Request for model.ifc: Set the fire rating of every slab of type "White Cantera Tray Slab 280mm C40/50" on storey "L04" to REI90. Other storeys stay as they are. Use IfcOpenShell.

First a look at what the model holds.

```python
import ifcopenshell
import ifcopenshell.util.element

model = ifcopenshell.open("model.ifc")
print(model.schema)
storey = next(s for s in model.by_type("IfcBuildingStorey") if s.Name == "L04")
slabs = [e for e in ifcopenshell.util.element.get_decomposition(storey) if e.is_a("IfcSlab")]
seen = {}
for e in slabs:
    element_type = ifcopenshell.util.element.get_type(e)
    key = (element_type.Name if element_type != e and element_type else None, ifcopenshell.util.element.get_pset(e, "Pset_SlabCommon", "FireRating"))
    seen[key] = seen.get(key, 0) + 1
for (name, value), count in sorted(seen.items(), key=str):
    print(count, "x", name, "|", value)
```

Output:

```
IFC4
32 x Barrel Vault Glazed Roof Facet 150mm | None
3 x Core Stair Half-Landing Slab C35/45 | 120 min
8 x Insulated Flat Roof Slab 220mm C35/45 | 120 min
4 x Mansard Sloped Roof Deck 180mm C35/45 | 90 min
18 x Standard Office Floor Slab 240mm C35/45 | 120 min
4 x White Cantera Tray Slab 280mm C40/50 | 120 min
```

```python
import ifcopenshell
import ifcopenshell.api.pset
import ifcopenshell.util.element

model = ifcopenshell.open("model.ifc")

storey = next(s for s in model.by_type("IfcBuildingStorey") if s.Name == "L04")
slabs = [e for e in ifcopenshell.util.element.get_decomposition(storey) if e.is_a("IfcSlab")]

count = 0
for e in slabs:
    element_type = ifcopenshell.util.element.get_type(e)
    if element_type in (None, e) or element_type.Name != "White Cantera Tray Slab 280mm C40/50":
        continue
    # add_pset returns the element's existing set when there is one.
    pset = ifcopenshell.api.pset.add_pset(model, product=e, name="Pset_SlabCommon")
    ifcopenshell.api.pset.edit_pset(model, pset=pset, properties={"FireRating": "REI90"})
    count += 1

print(count, "slabs updated")

model.write("model_updated.ifc")
```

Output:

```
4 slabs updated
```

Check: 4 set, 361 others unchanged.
